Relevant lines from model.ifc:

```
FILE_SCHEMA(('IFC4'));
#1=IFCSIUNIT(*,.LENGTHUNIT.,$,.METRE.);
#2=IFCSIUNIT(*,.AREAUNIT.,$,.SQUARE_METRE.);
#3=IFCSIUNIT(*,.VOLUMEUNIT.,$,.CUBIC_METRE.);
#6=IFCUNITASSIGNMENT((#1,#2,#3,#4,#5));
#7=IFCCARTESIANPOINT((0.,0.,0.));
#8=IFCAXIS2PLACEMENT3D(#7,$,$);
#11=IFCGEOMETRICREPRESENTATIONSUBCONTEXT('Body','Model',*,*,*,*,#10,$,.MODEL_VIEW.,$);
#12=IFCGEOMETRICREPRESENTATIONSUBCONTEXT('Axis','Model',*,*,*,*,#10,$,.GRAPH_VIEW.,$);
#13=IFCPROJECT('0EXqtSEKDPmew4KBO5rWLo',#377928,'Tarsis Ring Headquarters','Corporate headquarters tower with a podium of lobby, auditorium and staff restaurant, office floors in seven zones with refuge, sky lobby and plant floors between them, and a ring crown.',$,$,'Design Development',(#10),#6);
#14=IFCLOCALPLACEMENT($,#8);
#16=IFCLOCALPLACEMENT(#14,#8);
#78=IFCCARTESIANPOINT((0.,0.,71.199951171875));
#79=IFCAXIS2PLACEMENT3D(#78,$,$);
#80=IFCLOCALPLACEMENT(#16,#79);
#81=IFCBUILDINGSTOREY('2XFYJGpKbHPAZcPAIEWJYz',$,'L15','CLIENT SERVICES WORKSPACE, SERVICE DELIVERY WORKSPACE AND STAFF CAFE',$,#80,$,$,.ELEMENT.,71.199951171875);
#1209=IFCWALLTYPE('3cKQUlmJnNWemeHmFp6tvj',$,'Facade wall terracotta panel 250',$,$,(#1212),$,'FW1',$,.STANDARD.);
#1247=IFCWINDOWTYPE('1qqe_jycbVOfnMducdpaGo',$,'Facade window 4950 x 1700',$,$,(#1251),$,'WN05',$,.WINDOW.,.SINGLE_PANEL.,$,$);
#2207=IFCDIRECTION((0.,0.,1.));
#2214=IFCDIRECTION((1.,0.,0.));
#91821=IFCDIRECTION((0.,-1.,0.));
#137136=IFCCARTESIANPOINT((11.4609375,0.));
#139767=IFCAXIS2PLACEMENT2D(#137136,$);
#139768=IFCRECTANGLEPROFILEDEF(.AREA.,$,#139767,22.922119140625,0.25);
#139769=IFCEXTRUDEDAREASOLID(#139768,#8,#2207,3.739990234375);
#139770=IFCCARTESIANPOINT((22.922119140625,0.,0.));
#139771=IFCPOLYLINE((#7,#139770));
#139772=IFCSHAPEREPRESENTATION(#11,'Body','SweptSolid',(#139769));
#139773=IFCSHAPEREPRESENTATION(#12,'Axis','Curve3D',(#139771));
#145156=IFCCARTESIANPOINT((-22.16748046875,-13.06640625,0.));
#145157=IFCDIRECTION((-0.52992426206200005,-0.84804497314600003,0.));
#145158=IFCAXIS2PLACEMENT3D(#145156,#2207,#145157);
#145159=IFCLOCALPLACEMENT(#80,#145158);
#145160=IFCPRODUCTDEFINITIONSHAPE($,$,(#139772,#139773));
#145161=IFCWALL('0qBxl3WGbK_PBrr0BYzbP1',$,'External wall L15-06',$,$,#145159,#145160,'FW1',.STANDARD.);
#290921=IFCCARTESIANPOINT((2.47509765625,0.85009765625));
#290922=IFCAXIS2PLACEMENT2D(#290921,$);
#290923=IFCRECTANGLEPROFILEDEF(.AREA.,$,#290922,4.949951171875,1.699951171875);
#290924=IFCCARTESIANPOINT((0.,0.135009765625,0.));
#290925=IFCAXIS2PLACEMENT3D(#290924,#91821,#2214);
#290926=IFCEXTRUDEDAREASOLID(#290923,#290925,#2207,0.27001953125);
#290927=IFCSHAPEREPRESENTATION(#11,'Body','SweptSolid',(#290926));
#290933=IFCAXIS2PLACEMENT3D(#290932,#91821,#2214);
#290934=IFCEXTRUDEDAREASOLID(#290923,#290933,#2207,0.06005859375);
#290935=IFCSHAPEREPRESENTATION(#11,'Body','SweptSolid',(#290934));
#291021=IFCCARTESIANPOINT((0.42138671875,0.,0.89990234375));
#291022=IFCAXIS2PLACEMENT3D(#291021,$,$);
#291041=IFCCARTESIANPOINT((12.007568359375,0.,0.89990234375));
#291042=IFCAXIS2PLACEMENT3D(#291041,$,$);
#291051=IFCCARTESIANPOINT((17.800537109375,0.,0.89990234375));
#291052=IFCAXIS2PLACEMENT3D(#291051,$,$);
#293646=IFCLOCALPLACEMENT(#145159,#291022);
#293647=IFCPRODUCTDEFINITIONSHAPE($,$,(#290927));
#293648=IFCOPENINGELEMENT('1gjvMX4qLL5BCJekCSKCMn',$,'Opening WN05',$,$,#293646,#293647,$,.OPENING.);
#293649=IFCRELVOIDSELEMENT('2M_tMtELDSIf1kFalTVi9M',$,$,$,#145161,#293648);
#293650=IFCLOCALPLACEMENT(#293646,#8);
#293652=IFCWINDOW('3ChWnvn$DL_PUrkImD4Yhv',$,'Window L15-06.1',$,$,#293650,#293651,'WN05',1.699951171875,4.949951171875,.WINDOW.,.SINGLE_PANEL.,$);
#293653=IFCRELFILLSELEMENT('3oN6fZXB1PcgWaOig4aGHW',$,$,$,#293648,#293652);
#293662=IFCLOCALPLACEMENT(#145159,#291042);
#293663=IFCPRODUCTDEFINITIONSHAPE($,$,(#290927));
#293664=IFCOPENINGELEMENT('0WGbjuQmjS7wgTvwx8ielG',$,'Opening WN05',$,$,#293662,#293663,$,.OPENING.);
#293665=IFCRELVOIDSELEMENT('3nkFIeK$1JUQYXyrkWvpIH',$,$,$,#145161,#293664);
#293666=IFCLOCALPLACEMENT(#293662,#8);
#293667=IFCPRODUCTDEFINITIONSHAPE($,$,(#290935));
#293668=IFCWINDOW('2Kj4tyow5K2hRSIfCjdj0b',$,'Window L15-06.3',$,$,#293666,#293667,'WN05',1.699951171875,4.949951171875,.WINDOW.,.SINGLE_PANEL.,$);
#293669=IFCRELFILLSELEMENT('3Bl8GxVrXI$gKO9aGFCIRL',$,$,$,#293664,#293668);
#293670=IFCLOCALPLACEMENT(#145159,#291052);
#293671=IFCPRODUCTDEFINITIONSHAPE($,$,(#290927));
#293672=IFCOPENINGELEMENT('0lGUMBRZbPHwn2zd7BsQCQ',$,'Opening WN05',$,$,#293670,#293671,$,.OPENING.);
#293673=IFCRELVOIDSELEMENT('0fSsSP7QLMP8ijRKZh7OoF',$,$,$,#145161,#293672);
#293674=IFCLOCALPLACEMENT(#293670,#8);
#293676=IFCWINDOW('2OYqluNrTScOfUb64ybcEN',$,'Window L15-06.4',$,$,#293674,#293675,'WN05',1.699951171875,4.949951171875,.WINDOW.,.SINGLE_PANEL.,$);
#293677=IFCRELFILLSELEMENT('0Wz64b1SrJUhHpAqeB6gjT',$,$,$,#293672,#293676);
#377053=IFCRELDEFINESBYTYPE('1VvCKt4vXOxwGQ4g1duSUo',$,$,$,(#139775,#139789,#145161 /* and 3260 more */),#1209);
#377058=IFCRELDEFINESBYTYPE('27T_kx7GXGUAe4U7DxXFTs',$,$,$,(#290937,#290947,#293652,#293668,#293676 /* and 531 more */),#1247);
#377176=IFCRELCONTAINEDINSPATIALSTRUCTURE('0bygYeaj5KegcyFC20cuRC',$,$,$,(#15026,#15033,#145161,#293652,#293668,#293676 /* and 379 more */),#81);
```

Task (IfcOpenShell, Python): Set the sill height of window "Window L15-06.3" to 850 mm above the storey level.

```python
import numpy as np
import ifcopenshell
import ifcopenshell.api.geometry
import ifcopenshell.geom
import ifcopenshell.util.element
import ifcopenshell.util.placement
import ifcopenshell.util.shape
import ifcopenshell.util.unit

model = ifcopenshell.open("model.ifc")
unit_scale = ifcopenshell.util.unit.calculate_unit_scale(model)

window = model.by_guid("2Kj4tyow5K2hRSIfCjdj0b")
opening = window.FillsVoids[0].RelatingOpeningElement
storey = ifcopenshell.util.element.get_container(window, ifc_class="IfcBuildingStorey")
level = ifcopenshell.util.placement.get_local_placement(storey.ObjectPlacement)[2, 3]

# The opening's origin need not be at the sill, so measure its lowest point.
shape = ifcopenshell.geom.create_shape(ifcopenshell.geom.settings(), opening)
bottom = ifcopenshell.util.shape.get_shape_bottom_elevation(shape, shape.geometry) / unit_scale
dz = level + 0.85 - bottom

shift = np.array([0.0, 0.0, dz])
# The window is placed relative to its opening, so it follows when the opening moves.
matrix = ifcopenshell.util.placement.get_local_placement(opening.ObjectPlacement)
matrix[:3, 3] += shift
ifcopenshell.api.geometry.edit_object_placement(
    model, product=opening, matrix=matrix, is_si=False, should_transform_children=True
)

print(f"moved by {dz * unit_scale:+.3f} m")

model.write("model_v2.ifc")
```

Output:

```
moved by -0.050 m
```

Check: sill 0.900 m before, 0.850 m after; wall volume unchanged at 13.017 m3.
